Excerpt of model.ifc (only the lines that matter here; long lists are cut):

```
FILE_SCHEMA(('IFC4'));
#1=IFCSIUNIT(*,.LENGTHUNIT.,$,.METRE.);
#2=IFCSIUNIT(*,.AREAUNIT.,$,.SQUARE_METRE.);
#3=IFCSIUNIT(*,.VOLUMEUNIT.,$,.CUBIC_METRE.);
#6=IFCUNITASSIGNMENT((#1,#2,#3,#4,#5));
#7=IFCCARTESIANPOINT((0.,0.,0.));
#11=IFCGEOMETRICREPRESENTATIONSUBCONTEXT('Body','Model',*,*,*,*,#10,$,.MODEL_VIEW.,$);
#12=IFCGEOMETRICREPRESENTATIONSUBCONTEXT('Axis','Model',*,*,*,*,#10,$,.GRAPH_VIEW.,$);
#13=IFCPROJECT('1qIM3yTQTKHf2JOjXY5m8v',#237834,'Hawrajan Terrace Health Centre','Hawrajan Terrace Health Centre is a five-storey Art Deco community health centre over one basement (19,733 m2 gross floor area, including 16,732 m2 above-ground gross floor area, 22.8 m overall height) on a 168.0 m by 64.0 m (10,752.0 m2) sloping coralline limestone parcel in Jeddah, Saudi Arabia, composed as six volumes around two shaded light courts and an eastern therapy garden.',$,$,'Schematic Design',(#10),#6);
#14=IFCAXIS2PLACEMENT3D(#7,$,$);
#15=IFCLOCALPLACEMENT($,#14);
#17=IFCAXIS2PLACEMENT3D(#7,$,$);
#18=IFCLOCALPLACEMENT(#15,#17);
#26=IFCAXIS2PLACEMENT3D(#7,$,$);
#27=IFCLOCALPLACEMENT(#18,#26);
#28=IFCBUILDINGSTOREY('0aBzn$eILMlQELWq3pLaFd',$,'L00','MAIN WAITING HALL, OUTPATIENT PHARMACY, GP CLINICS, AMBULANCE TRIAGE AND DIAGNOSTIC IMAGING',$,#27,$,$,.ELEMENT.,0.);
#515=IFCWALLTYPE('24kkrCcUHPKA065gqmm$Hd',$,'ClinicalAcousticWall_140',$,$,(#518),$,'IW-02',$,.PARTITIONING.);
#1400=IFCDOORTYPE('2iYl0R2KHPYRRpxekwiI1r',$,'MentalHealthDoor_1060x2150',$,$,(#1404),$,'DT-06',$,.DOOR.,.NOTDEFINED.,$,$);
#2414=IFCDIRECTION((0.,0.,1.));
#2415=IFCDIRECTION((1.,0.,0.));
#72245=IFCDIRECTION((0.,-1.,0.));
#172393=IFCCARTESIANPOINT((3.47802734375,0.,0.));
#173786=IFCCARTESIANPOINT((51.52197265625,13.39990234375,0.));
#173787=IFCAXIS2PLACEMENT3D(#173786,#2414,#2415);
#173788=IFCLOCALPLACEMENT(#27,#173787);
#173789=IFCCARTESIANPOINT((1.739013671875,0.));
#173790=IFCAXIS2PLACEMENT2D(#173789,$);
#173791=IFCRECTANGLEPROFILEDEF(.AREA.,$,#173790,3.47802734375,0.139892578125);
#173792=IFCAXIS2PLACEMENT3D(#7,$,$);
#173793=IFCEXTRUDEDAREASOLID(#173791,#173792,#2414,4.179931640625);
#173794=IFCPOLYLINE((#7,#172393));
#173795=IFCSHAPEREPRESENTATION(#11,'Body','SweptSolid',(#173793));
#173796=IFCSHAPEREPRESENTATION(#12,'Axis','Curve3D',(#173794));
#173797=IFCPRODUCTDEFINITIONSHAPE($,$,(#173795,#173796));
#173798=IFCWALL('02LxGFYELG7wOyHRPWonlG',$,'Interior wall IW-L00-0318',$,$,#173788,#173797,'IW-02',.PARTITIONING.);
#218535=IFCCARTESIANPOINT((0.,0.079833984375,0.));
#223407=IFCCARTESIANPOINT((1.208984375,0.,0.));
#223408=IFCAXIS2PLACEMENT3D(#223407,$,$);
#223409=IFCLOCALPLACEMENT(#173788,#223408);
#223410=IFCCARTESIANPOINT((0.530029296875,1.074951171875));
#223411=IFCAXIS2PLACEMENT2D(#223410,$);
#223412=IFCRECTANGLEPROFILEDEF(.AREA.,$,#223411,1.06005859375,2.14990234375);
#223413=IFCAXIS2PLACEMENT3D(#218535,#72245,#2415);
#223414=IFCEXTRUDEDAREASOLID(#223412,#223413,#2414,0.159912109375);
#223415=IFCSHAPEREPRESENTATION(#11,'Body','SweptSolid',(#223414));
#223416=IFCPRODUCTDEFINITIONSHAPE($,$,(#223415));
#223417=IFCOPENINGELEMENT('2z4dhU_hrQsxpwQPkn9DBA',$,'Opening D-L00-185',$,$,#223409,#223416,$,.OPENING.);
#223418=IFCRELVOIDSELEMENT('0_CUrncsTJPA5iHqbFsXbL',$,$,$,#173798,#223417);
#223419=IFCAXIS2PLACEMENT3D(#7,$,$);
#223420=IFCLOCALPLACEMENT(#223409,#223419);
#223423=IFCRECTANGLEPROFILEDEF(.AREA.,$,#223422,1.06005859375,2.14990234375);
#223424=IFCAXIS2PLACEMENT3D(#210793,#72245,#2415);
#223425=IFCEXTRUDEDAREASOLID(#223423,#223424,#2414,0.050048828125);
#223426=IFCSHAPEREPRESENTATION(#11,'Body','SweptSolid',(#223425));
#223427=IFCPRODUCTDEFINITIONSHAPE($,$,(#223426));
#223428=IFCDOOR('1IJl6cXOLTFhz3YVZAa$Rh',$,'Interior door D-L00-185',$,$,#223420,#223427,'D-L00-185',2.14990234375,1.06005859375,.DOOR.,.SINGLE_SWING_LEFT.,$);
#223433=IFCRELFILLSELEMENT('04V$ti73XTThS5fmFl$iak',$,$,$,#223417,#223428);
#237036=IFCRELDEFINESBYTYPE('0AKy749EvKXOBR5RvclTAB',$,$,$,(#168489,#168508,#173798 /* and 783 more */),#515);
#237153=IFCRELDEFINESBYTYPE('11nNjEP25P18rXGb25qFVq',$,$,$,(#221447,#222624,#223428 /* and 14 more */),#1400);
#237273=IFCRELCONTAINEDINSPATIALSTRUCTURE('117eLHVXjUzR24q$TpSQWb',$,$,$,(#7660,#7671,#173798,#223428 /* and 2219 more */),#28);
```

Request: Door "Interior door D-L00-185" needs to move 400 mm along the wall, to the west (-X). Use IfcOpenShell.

```python
import ifcopenshell
import ifcopenshell.api.geometry
import ifcopenshell.util.placement
import ifcopenshell.util.unit

model = ifcopenshell.open("model.ifc")
unit_scale = ifcopenshell.util.unit.calculate_unit_scale(model)

door = model.by_guid("1IJl6cXOLTFhz3YVZAa$Rh")
opening = door.FillsVoids[0].RelatingOpeningElement
wall = opening.VoidsElements[0].RelatingBuildingElement

wall_matrix = ifcopenshell.util.placement.get_local_placement(wall.ObjectPlacement)
shift = wall_matrix[:3, 0] * -0.4 / unit_scale
before = ifcopenshell.util.placement.get_local_placement(door.ObjectPlacement)[:3, 3].copy()

# The door is placed relative to its opening, so it follows when the opening moves.
matrix = ifcopenshell.util.placement.get_local_placement(opening.ObjectPlacement)
matrix[:3, 3] += shift
ifcopenshell.api.geometry.edit_object_placement(
    model, product=opening, matrix=matrix, is_si=False, should_transform_children=True
)

after = ifcopenshell.util.placement.get_local_placement(door.ObjectPlacement)[:3, 3]
print("door moved by", (after - before).round(3) + 0.0)

model.write("model_rev.ifc")
```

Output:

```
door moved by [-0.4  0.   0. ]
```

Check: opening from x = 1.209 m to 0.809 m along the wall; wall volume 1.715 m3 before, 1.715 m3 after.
